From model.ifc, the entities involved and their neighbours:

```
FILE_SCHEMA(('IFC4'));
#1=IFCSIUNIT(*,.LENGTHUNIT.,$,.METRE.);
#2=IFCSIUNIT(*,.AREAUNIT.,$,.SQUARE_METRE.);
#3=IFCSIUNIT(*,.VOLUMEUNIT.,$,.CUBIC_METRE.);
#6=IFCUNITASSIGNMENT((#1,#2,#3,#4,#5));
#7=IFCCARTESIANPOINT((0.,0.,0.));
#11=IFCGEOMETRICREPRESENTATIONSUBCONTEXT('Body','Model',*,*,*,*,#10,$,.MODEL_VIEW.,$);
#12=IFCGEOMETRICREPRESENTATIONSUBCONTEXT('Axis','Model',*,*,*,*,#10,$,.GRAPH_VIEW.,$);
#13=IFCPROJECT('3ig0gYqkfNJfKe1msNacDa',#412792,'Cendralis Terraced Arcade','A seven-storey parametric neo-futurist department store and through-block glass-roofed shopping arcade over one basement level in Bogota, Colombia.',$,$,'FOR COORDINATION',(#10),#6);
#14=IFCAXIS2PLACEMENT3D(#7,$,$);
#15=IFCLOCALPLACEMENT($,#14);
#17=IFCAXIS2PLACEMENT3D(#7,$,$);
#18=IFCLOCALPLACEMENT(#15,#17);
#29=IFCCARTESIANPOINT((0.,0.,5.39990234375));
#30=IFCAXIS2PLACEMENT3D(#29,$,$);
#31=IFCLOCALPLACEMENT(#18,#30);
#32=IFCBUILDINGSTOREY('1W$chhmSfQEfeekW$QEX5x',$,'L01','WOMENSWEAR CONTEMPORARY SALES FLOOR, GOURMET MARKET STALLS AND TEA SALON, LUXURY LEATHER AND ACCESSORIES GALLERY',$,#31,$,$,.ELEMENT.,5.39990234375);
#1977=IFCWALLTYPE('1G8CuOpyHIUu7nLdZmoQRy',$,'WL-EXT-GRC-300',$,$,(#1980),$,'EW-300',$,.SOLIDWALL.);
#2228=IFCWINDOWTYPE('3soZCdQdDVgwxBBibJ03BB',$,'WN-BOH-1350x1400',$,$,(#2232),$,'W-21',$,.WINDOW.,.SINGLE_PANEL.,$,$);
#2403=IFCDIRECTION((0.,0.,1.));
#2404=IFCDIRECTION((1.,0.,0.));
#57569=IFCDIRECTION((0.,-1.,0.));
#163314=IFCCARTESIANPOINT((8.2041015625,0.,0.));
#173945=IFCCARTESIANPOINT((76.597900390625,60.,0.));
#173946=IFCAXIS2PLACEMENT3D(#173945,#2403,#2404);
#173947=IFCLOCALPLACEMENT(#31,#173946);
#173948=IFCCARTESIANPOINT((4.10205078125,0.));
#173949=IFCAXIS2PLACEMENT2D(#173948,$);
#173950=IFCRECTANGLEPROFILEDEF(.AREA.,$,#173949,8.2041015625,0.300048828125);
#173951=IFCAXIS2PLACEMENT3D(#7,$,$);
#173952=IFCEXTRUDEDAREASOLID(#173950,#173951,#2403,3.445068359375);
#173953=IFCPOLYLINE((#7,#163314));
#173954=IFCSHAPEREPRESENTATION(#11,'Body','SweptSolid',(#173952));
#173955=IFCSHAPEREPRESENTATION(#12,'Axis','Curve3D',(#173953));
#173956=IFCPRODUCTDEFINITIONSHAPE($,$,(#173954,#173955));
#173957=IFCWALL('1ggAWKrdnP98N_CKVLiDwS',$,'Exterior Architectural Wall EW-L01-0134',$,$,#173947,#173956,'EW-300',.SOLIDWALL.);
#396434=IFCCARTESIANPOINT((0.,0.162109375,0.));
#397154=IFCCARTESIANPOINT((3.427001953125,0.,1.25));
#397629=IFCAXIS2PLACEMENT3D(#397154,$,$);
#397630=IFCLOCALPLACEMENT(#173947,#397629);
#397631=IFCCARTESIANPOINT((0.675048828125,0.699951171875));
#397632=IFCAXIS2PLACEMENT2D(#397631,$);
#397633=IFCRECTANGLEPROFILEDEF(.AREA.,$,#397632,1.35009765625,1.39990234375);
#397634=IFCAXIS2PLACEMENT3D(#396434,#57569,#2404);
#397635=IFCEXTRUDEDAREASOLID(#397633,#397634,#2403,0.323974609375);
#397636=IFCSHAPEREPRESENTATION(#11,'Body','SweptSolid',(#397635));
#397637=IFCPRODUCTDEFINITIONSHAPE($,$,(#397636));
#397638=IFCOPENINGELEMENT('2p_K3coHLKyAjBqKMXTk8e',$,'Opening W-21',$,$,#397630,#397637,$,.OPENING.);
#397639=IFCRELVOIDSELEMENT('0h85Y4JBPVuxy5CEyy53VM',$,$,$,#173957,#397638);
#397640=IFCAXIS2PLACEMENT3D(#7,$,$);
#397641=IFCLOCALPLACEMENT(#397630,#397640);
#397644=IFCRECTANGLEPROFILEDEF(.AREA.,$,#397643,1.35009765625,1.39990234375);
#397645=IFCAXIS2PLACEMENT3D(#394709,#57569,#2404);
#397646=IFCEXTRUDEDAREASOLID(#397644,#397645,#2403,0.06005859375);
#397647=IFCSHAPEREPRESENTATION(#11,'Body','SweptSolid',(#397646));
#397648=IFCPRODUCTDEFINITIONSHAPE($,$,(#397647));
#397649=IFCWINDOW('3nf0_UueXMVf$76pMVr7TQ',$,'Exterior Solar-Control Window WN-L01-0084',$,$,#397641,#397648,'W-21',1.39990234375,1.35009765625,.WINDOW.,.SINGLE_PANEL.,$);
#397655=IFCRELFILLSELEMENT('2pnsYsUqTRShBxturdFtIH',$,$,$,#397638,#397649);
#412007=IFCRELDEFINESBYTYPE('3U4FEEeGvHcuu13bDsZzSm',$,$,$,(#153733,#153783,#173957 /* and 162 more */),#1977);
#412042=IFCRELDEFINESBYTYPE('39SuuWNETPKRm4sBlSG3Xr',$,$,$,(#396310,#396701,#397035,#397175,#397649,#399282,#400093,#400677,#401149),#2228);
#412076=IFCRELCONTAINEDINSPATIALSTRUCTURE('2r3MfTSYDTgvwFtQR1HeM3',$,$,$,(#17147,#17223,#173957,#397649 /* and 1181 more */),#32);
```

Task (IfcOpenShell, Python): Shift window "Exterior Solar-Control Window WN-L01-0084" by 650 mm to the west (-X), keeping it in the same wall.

```python
import ifcopenshell
import ifcopenshell.api.geometry
import ifcopenshell.util.placement

model = ifcopenshell.open("model.ifc")

window = model.by_id(397649)
opening = window.FillsVoids[0].RelatingOpeningElement
wall = opening.VoidsElements[0].RelatingBuildingElement

wall_matrix = ifcopenshell.util.placement.get_local_placement(wall.ObjectPlacement)
shift = wall_matrix[:3, 0] * -0.65
before = ifcopenshell.util.placement.get_local_placement(window.ObjectPlacement)[:3, 3].copy()

# The window is placed relative to its opening, so it follows when the opening moves.
matrix = ifcopenshell.util.placement.get_local_placement(opening.ObjectPlacement)
matrix[:3, 3] += shift
ifcopenshell.api.geometry.edit_object_placement(
    model, product=opening, matrix=matrix, is_si=False, should_transform_children=True
)

after = ifcopenshell.util.placement.get_local_placement(window.ObjectPlacement)[:3, 3]
print("window moved by", (after - before).round(3) + 0.0)

model.write("model_v2.ifc")
```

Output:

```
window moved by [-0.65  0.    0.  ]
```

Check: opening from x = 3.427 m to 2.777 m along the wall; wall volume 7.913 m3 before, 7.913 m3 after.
